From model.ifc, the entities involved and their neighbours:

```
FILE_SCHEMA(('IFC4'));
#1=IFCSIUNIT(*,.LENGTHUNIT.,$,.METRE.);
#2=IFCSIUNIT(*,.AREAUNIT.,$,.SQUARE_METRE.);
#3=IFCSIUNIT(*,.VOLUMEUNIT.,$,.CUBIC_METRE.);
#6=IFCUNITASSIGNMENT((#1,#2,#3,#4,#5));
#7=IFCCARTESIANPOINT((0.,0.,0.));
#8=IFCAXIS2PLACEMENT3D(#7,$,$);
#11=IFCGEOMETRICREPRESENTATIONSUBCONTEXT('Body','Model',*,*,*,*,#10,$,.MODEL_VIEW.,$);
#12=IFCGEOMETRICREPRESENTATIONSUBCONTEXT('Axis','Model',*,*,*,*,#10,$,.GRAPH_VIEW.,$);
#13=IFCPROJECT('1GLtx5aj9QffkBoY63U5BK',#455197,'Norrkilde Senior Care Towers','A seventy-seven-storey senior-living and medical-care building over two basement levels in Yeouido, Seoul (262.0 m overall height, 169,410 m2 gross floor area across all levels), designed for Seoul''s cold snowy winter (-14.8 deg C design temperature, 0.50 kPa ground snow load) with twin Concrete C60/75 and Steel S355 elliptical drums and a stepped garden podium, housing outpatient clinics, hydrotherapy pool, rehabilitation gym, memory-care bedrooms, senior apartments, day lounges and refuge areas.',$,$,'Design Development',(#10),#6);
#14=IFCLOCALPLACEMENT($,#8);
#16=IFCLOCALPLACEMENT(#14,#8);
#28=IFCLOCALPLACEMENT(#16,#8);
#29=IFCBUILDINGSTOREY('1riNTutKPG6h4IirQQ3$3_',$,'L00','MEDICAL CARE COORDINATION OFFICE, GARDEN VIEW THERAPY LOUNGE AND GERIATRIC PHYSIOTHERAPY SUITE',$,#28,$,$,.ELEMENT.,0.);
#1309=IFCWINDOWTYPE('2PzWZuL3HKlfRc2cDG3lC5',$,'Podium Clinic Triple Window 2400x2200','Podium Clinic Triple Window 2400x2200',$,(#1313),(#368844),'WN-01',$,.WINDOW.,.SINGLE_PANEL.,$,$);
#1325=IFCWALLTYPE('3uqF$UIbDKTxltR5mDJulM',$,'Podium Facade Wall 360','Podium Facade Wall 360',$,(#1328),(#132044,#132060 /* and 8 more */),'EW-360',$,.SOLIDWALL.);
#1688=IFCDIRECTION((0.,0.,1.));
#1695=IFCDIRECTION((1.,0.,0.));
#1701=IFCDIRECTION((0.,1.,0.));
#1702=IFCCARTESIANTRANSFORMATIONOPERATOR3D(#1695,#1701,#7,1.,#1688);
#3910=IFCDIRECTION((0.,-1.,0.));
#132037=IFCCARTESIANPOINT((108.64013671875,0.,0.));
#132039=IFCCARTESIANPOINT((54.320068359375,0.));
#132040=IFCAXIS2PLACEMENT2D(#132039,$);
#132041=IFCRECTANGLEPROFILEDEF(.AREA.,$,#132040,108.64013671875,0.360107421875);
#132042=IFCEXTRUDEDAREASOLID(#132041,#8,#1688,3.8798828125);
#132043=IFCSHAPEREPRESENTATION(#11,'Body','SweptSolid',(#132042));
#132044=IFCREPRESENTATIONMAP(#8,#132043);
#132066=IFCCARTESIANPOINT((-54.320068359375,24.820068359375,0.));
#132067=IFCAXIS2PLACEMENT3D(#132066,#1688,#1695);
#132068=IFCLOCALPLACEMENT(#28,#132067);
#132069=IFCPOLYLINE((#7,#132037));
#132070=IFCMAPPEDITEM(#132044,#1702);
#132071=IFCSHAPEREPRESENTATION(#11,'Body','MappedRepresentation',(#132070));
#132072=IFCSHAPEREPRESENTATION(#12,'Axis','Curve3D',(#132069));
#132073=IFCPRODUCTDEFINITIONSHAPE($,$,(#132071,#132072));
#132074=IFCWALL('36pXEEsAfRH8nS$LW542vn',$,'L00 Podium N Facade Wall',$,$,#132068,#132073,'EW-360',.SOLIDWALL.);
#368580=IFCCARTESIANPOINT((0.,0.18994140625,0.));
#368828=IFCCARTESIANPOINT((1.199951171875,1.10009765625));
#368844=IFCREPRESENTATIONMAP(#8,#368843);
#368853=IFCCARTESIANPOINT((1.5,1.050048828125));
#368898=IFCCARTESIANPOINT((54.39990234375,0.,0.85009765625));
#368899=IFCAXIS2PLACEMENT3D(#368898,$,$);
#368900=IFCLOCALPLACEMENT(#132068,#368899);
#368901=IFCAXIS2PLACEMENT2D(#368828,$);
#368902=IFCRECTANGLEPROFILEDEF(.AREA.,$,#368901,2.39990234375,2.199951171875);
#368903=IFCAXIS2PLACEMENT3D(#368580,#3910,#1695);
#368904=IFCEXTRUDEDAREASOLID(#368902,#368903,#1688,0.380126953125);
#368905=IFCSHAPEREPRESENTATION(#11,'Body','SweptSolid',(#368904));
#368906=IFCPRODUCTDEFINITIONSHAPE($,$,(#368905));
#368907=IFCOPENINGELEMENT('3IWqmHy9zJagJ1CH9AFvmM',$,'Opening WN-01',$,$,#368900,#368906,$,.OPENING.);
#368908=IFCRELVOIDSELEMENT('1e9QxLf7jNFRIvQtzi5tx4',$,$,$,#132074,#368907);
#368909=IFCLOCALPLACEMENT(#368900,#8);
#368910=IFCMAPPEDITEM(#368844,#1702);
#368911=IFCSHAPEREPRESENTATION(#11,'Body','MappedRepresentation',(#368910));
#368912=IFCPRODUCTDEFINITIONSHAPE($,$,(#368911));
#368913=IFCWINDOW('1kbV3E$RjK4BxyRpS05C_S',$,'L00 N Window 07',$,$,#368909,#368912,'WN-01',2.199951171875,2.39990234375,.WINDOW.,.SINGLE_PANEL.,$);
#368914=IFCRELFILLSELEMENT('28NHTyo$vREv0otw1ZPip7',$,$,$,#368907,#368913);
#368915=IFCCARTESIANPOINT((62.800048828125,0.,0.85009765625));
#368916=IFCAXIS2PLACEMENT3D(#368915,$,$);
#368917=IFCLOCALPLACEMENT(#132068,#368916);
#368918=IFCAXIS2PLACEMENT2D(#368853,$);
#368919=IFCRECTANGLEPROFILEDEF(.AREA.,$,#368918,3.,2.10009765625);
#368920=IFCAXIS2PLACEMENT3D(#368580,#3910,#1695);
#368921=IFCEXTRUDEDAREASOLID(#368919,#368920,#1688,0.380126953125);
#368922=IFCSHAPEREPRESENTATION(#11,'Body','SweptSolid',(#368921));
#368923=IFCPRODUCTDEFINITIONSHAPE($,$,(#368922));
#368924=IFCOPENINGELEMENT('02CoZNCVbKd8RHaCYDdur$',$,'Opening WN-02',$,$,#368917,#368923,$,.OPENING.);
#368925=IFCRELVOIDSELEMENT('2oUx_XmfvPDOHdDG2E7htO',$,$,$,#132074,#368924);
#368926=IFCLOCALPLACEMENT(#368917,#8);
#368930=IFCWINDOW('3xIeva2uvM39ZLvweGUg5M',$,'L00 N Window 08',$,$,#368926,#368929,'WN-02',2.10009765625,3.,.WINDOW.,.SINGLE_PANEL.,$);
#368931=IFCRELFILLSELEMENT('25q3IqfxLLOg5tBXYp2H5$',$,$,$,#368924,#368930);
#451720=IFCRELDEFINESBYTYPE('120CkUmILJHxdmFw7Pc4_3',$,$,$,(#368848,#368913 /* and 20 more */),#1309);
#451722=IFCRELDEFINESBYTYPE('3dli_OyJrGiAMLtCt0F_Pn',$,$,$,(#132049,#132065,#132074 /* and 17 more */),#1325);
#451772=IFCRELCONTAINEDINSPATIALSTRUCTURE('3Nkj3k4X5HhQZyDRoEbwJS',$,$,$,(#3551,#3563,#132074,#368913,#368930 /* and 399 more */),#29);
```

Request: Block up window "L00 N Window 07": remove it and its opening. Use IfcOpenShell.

```python
import ifcopenshell
import ifcopenshell.api.feature
import ifcopenshell.api.root
import ifcopenshell.geom
import ifcopenshell.util.shape

model = ifcopenshell.open("model.ifc")
settings = ifcopenshell.geom.settings()


def volume(element):
    """Net volume in cubic metres, openings subtracted."""
    shape = ifcopenshell.geom.create_shape(settings, element)
    return ifcopenshell.util.shape.get_volume(shape.geometry)


window = model.by_id(368913)
opening = window.FillsVoids[0].RelatingOpeningElement
wall = opening.VoidsElements[0].RelatingBuildingElement
before = volume(wall)

ifcopenshell.api.root.remove_product(model, product=window)
ifcopenshell.api.feature.remove_feature(model, feature=opening)

after = volume(wall)

print(f"wall volume {before:.3f} -> {after:.3f} m3")

model.write("model_v2.ifc")
```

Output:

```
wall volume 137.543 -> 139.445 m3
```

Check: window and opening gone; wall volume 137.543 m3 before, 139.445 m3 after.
